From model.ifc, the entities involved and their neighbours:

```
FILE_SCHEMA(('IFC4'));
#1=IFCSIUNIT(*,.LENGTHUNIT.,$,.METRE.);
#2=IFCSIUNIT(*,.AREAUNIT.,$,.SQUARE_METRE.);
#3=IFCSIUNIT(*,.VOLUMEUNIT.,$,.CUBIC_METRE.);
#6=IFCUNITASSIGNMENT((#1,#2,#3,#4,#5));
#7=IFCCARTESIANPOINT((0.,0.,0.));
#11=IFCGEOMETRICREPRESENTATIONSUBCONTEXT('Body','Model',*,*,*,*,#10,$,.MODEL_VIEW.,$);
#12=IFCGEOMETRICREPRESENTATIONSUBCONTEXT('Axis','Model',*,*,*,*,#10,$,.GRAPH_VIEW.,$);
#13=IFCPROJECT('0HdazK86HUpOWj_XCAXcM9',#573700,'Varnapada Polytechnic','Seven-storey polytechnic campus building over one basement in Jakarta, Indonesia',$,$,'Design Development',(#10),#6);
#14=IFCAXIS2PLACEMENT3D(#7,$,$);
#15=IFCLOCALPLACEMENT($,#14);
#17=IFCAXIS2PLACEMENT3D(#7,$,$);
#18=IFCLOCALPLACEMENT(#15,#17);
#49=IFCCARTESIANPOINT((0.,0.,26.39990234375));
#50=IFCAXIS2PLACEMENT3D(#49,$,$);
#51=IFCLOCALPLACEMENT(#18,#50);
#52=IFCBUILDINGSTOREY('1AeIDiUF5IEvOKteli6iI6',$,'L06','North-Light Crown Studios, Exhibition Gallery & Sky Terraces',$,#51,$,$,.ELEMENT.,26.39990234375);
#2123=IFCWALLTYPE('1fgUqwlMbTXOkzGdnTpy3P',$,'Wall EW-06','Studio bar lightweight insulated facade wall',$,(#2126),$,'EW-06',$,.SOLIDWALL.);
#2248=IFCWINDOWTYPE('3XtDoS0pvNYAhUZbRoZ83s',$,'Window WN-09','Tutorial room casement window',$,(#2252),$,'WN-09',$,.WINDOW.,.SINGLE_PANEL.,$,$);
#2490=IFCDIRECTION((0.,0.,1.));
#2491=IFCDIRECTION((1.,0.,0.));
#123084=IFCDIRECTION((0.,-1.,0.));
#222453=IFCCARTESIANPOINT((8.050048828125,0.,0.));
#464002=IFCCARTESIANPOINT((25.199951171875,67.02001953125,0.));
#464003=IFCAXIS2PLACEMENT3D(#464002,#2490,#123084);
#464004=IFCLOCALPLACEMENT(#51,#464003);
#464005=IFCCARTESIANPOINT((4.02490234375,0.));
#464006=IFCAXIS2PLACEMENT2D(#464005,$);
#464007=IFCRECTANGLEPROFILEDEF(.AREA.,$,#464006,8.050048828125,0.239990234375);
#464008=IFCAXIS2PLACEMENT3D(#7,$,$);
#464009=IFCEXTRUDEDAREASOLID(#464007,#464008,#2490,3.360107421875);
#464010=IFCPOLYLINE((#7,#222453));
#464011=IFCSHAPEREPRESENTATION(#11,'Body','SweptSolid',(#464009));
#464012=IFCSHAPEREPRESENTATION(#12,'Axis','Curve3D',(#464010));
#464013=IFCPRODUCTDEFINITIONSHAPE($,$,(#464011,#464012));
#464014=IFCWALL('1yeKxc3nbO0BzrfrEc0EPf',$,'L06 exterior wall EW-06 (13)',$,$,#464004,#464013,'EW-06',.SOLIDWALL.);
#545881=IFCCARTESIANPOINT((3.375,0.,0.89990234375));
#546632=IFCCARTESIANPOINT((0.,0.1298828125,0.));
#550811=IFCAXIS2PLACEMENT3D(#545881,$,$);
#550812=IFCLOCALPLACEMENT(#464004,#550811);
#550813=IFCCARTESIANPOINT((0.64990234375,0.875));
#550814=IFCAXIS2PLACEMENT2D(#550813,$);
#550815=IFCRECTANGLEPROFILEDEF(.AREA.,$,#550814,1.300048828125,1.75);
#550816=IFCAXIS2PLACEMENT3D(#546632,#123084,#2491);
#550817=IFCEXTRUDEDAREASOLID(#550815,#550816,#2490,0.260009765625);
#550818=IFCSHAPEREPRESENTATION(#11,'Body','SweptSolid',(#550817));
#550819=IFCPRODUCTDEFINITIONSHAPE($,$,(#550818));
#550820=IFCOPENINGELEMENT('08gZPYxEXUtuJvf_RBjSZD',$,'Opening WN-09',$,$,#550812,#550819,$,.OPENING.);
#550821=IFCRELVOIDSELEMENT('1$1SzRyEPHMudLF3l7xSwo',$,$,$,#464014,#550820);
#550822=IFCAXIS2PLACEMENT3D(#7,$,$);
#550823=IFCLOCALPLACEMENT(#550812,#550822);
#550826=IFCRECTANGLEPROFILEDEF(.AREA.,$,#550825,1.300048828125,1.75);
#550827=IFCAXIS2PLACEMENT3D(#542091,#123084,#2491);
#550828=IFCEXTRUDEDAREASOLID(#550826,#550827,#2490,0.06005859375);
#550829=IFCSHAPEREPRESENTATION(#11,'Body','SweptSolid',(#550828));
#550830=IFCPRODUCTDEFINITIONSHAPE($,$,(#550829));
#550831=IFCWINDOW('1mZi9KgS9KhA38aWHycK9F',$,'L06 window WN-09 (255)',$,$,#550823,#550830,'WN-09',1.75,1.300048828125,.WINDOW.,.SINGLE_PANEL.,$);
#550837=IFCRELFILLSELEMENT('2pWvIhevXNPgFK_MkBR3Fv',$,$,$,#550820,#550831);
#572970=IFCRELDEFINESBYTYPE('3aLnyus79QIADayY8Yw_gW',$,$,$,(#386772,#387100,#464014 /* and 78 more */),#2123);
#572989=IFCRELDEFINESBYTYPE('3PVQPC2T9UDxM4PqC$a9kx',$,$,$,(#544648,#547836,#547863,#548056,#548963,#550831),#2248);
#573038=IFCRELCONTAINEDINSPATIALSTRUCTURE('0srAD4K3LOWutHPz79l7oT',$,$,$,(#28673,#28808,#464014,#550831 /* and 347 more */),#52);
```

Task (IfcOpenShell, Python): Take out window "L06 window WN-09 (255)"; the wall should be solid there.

```python
import ifcopenshell
import ifcopenshell.api.feature
import ifcopenshell.api.root
import ifcopenshell.geom
import ifcopenshell.util.shape

model = ifcopenshell.open("model.ifc")
settings = ifcopenshell.geom.settings()


def volume(element):
    """Net volume in cubic metres, openings subtracted."""
    shape = ifcopenshell.geom.create_shape(settings, element)
    return ifcopenshell.util.shape.get_volume(shape.geometry)


window = model.by_id(550831)
opening = window.FillsVoids[0].RelatingOpeningElement
wall = opening.VoidsElements[0].RelatingBuildingElement
before = volume(wall)

ifcopenshell.api.root.remove_product(model, product=window)
ifcopenshell.api.feature.remove_feature(model, feature=opening)

after = volume(wall)

print(f"wall volume {before:.3f} -> {after:.3f} m3")

model.write("model_edited.ifc")
```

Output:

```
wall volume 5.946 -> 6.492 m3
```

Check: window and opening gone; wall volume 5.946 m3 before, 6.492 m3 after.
